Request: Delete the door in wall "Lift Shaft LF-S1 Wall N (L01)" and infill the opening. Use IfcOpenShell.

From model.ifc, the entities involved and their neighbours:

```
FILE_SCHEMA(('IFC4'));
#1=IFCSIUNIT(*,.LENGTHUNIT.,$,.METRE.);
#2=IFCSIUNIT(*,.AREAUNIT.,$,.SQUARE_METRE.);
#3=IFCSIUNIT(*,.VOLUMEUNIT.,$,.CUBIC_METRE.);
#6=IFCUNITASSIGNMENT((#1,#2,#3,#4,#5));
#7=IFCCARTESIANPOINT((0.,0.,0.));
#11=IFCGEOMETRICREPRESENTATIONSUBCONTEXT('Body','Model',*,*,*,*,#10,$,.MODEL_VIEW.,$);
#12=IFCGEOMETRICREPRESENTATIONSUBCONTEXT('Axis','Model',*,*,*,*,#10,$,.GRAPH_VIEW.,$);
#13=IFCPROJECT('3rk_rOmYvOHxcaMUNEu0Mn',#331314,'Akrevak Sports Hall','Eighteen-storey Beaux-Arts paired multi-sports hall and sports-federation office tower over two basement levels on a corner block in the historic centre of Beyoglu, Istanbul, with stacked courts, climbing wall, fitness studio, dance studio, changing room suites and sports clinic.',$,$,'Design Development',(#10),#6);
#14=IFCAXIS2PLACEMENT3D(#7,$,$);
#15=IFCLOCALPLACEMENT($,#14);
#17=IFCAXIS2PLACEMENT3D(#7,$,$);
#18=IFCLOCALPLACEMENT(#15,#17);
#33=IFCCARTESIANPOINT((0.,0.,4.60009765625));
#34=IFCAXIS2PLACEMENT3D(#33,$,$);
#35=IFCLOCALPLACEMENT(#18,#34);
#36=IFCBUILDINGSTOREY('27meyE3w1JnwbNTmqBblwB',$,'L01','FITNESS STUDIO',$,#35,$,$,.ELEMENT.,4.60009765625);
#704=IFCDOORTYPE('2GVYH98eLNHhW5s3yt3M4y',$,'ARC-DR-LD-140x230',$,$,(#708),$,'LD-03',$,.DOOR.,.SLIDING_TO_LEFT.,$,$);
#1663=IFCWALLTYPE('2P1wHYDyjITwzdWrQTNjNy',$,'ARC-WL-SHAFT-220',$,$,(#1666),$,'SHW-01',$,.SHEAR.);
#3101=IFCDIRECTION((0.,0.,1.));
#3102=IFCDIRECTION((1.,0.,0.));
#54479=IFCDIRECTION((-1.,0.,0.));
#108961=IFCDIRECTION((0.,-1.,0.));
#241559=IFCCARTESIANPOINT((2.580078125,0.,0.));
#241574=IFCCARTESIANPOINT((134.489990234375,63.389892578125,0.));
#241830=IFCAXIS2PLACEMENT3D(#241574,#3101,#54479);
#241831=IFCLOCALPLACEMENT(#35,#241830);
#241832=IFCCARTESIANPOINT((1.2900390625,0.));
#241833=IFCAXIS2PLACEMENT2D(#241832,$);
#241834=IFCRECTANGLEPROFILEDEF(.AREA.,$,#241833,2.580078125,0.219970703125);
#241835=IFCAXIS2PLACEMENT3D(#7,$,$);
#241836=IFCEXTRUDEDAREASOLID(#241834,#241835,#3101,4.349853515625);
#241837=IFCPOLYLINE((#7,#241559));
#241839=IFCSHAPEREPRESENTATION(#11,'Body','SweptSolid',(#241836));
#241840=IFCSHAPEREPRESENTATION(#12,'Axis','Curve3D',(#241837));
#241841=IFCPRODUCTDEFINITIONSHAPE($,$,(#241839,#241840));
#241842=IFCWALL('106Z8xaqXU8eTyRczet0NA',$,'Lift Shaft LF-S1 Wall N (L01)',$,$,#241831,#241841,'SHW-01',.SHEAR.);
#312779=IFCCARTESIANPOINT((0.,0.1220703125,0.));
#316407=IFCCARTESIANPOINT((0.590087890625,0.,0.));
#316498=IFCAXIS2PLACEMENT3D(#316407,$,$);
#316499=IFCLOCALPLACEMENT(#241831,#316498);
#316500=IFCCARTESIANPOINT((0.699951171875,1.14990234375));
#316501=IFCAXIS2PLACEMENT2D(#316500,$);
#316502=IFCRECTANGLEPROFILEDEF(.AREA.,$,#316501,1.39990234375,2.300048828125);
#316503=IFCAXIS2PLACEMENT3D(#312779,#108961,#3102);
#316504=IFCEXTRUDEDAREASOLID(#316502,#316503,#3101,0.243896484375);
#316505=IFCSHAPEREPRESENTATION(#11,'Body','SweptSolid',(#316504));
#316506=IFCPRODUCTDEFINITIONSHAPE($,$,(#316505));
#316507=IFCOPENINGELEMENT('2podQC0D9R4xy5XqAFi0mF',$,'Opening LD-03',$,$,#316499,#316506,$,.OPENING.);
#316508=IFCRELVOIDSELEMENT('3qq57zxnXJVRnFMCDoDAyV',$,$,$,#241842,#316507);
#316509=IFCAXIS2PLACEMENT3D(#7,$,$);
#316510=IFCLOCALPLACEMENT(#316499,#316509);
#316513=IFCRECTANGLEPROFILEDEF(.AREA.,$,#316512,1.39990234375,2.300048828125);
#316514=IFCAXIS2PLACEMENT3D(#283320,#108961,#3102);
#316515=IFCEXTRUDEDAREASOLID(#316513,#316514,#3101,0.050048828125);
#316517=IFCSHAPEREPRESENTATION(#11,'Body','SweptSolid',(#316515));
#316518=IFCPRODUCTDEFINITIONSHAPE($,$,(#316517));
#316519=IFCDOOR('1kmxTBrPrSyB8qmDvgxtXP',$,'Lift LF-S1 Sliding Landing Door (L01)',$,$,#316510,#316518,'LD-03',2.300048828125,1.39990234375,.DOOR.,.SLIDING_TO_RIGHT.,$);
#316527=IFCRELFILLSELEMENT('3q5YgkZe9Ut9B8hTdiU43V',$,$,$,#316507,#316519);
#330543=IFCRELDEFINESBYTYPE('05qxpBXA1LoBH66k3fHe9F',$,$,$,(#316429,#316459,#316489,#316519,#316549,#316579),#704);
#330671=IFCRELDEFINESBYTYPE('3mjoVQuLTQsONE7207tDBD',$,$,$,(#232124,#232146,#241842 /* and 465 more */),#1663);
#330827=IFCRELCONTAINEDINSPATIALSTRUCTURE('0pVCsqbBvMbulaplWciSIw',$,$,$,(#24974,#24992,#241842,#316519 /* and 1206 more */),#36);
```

```python
import ifcopenshell
import ifcopenshell.api.feature
import ifcopenshell.api.root
import ifcopenshell.geom
import ifcopenshell.util.shape

model = ifcopenshell.open("model.ifc")
settings = ifcopenshell.geom.settings()


def volume(element):
    """Net volume in cubic metres, openings subtracted."""
    shape = ifcopenshell.geom.create_shape(settings, element)
    return ifcopenshell.util.shape.get_volume(shape.geometry)


door = model.by_id(316519)
opening = door.FillsVoids[0].RelatingOpeningElement
wall = opening.VoidsElements[0].RelatingBuildingElement
before = volume(wall)

ifcopenshell.api.root.remove_product(model, product=door)
ifcopenshell.api.feature.remove_feature(model, feature=opening)

after = volume(wall)

print(f"wall volume {before:.3f} -> {after:.3f} m3")

model.write("model_rev.ifc")
```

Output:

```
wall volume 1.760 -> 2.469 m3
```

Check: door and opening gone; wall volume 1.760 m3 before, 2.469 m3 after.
